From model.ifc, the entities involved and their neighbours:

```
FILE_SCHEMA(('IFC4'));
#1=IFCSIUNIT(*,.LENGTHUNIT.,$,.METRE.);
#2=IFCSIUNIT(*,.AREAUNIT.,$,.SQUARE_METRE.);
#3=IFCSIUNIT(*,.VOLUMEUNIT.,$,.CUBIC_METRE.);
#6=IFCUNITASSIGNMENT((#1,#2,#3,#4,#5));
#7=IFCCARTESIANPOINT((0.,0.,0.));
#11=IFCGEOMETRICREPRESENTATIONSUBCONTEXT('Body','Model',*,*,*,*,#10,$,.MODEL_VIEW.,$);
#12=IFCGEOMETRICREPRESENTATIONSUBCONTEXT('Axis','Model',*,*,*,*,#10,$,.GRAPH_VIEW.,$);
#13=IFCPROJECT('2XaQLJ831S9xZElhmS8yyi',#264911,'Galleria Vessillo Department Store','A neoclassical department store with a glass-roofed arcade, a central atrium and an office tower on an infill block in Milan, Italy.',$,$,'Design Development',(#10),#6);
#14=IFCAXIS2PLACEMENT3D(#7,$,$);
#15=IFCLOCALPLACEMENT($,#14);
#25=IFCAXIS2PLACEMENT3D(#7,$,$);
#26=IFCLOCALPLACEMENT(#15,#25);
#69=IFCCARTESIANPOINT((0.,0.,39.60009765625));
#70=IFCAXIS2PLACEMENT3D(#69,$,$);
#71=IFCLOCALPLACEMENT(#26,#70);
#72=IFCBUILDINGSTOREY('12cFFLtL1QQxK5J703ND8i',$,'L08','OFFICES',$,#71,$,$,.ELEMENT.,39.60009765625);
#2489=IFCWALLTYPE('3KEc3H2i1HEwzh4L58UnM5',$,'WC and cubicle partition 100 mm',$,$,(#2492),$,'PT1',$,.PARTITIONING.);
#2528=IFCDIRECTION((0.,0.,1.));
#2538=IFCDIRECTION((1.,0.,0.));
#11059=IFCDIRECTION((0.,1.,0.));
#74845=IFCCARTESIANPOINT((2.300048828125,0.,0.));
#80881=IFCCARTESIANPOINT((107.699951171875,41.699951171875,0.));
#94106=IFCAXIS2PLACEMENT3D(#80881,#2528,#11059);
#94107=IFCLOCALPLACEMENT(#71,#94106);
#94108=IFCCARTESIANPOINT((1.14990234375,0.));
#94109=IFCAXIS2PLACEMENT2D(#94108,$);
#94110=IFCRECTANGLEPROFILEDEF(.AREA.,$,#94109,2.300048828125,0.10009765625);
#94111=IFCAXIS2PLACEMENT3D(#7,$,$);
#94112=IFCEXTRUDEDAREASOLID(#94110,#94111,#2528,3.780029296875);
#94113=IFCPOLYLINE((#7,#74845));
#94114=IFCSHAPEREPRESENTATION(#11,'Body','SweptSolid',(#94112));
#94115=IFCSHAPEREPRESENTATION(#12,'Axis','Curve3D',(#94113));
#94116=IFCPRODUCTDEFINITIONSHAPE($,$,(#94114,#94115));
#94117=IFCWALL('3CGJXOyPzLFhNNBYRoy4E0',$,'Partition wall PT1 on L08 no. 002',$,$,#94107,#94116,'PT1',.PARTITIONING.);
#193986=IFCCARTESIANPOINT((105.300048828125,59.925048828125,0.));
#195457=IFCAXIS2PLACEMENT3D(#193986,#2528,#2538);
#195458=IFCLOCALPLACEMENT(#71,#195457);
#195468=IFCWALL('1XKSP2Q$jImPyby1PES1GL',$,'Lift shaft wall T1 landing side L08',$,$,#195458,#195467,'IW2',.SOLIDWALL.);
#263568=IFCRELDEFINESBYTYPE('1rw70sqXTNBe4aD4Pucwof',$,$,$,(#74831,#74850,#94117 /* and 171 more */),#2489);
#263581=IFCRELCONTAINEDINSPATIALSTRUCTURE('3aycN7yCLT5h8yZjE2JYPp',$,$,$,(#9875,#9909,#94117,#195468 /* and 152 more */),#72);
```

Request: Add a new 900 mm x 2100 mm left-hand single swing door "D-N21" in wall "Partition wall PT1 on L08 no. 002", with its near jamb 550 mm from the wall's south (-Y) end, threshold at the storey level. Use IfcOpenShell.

```python
import numpy as np
import ifcopenshell
import ifcopenshell.api.feature
import ifcopenshell.api.geometry
import ifcopenshell.api.root
import ifcopenshell.api.spatial
import ifcopenshell.geom
import ifcopenshell.util.element
import ifcopenshell.util.placement
import ifcopenshell.util.representation
import ifcopenshell.util.shape
import ifcopenshell.util.unit

model = ifcopenshell.open("model.ifc")
unit_scale = ifcopenshell.util.unit.calculate_unit_scale(model)
settings = ifcopenshell.geom.settings()


def volume(element):
    """Net volume in cubic metres, openings subtracted."""
    shape = ifcopenshell.geom.create_shape(settings, element)
    return ifcopenshell.util.shape.get_volume(shape.geometry)


wall = model.by_guid("3CGJXOyPzLFhNNBYRoy4E0")
storey = ifcopenshell.util.element.get_container(wall, ifc_class="IfcBuildingStorey")
context = ifcopenshell.util.representation.get_context(model, "Model", "Body", "MODEL_VIEW")
before = volume(wall)

width, height, from_end, sill = 0.9, 2.1, 0.55, 0.0  # metres

# The wall runs along its own X axis, and the end named is its -X end.
wall_shape = ifcopenshell.geom.create_shape(settings, wall)
x, y, z = ifcopenshell.util.shape.get_vertices(wall_shape.geometry).T
start = x.min() + from_end
face, thickness = float(y.min()), float(y.max() - y.min())
wall_matrix = ifcopenshell.util.placement.get_local_placement(wall.ObjectPlacement)
level = ifcopenshell.util.placement.get_local_placement(storey.ObjectPlacement)[2, 3]


def in_wall(x, y):
    """Placement at x, y metres in the wall's axes, at sill height."""
    matrix = wall_matrix.copy()
    matrix[:, 3] = wall_matrix @ np.array([x / unit_scale, y / unit_scale, 0.0, 1.0])
    matrix[2, 3] = level + sill / unit_scale
    return matrix


# Opening: a box that overshoots both wall faces by 50 mm.
opening = ifcopenshell.api.root.create_entity(model, ifc_class="IfcOpeningElement", predefined_type="OPENING")
box = ifcopenshell.api.geometry.add_wall_representation(
    model, context=context, length=width, height=height, thickness=thickness + 0.1
)
ifcopenshell.api.geometry.assign_representation(model, product=opening, representation=box)
ifcopenshell.api.geometry.edit_object_placement(model, product=opening, matrix=in_wall(start, face - 0.05), is_si=False)
ifcopenshell.api.feature.add_feature(model, feature=opening, element=wall)

door = ifcopenshell.api.root.create_entity(model, ifc_class="IfcDoor", name="D-N21", predefined_type="DOOR")
door.OverallWidth, door.OverallHeight = width / unit_scale, height / unit_scale
door.OperationType = "SINGLE_SWING_LEFT"
body = ifcopenshell.api.geometry.add_door_representation(
    model,
    context=context,
    overall_width=door.OverallWidth,
    overall_height=door.OverallHeight,
    operation_type="SINGLE_SWING_LEFT",
    lining_properties={"LiningDepth": thickness / unit_scale, "ThresholdDepth": thickness / unit_scale},
)
ifcopenshell.api.geometry.assign_representation(model, product=door, representation=body)
ifcopenshell.api.spatial.assign_container(model, products=[door], relating_structure=storey)
ifcopenshell.api.feature.add_filling(model, opening=opening, element=door)

# The lining spans the wall, so the door starts at the wall face.
ifcopenshell.api.geometry.edit_object_placement(model, product=door, matrix=in_wall(start, face), is_si=False)

after = volume(wall)

print(f"wall volume {before:.3f} -> {after:.3f} m3")

model.write("model_rev.ifc")
```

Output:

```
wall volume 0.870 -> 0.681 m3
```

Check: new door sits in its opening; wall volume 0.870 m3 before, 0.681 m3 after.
